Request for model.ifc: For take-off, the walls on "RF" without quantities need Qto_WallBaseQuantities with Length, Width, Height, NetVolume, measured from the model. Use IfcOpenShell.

First a look at what the model holds.

```python
import ifcopenshell
import ifcopenshell.util.element
import ifcopenshell.util.unit

model = ifcopenshell.open("model.ifc")
print(model.schema)
for unit_type in ("LENGTHUNIT", "AREAUNIT", "VOLUMEUNIT"):
    print(unit_type, ifcopenshell.util.unit.calculate_unit_scale(model, unit_type))
storey = next(s for s in model.by_type("IfcBuildingStorey") if s.Name == "RF")
walls = [e for e in ifcopenshell.util.element.get_decomposition(storey) if e.is_a("IfcWall")]
for e in sorted(walls, key=lambda e: e.id()):
    print(e.id(), e.is_a(), e.Name, list(ifcopenshell.util.element.get_psets(e, qtos_only=True)), sep=" | ")
```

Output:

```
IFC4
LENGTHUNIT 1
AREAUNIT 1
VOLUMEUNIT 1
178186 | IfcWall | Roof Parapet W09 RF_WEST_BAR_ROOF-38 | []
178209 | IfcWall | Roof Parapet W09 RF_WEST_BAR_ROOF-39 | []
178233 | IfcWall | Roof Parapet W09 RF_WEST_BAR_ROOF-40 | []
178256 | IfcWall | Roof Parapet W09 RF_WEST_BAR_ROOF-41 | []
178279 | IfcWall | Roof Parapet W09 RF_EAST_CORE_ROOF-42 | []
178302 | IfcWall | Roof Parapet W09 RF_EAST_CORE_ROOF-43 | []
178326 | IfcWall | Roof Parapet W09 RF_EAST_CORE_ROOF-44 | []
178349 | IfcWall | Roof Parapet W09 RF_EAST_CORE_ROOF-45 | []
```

```python
import ifcopenshell
import ifcopenshell.api.pset
import ifcopenshell.geom
import ifcopenshell.util.element
import ifcopenshell.util.shape
import ifcopenshell.util.unit

model = ifcopenshell.open("model.ifc")
unit_scale = ifcopenshell.util.unit.calculate_unit_scale(model)
volume_scale = ifcopenshell.util.unit.calculate_unit_scale(model, "VOLUMEUNIT")
settings = ifcopenshell.geom.settings()

storey = next(s for s in model.by_type("IfcBuildingStorey") if s.Name == "RF")
walls = [e for e in ifcopenshell.util.element.get_decomposition(storey) if e.is_a("IfcWall")]

for e in sorted(walls, key=lambda e: e.id()):
    if ifcopenshell.util.element.get_psets(e, qtos_only=True, should_inherit=False):
        continue
    # Geometry comes back in metres, in the element's own axes.
    shape = ifcopenshell.geom.create_shape(settings, e)
    values = {
        "Length": ifcopenshell.util.shape.get_x(shape.geometry) / unit_scale,
        "Width": ifcopenshell.util.shape.get_y(shape.geometry) / unit_scale,
        "Height": ifcopenshell.util.shape.get_z(shape.geometry) / unit_scale,
        "NetVolume": ifcopenshell.util.shape.get_volume(shape.geometry) / volume_scale,
    }
    qto = ifcopenshell.api.pset.add_qto(model, product=e, name="Qto_WallBaseQuantities")
    ifcopenshell.api.pset.edit_qto(model, qto=qto, properties=values)
    print(e.id(), {k: round(v, 3) for k, v in values.items()})

model.write("model_edited.ifc")
```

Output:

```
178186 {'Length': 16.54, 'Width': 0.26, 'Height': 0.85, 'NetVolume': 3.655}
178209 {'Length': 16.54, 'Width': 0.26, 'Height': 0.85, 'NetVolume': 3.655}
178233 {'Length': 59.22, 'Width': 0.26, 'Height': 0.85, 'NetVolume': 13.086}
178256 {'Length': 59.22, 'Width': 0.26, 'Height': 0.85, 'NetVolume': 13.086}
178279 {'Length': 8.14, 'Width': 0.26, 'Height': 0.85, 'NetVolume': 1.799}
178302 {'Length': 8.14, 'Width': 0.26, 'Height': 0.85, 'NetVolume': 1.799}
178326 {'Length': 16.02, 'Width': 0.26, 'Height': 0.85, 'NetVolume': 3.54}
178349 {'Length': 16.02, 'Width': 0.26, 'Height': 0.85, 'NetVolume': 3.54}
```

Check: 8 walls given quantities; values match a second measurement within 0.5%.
